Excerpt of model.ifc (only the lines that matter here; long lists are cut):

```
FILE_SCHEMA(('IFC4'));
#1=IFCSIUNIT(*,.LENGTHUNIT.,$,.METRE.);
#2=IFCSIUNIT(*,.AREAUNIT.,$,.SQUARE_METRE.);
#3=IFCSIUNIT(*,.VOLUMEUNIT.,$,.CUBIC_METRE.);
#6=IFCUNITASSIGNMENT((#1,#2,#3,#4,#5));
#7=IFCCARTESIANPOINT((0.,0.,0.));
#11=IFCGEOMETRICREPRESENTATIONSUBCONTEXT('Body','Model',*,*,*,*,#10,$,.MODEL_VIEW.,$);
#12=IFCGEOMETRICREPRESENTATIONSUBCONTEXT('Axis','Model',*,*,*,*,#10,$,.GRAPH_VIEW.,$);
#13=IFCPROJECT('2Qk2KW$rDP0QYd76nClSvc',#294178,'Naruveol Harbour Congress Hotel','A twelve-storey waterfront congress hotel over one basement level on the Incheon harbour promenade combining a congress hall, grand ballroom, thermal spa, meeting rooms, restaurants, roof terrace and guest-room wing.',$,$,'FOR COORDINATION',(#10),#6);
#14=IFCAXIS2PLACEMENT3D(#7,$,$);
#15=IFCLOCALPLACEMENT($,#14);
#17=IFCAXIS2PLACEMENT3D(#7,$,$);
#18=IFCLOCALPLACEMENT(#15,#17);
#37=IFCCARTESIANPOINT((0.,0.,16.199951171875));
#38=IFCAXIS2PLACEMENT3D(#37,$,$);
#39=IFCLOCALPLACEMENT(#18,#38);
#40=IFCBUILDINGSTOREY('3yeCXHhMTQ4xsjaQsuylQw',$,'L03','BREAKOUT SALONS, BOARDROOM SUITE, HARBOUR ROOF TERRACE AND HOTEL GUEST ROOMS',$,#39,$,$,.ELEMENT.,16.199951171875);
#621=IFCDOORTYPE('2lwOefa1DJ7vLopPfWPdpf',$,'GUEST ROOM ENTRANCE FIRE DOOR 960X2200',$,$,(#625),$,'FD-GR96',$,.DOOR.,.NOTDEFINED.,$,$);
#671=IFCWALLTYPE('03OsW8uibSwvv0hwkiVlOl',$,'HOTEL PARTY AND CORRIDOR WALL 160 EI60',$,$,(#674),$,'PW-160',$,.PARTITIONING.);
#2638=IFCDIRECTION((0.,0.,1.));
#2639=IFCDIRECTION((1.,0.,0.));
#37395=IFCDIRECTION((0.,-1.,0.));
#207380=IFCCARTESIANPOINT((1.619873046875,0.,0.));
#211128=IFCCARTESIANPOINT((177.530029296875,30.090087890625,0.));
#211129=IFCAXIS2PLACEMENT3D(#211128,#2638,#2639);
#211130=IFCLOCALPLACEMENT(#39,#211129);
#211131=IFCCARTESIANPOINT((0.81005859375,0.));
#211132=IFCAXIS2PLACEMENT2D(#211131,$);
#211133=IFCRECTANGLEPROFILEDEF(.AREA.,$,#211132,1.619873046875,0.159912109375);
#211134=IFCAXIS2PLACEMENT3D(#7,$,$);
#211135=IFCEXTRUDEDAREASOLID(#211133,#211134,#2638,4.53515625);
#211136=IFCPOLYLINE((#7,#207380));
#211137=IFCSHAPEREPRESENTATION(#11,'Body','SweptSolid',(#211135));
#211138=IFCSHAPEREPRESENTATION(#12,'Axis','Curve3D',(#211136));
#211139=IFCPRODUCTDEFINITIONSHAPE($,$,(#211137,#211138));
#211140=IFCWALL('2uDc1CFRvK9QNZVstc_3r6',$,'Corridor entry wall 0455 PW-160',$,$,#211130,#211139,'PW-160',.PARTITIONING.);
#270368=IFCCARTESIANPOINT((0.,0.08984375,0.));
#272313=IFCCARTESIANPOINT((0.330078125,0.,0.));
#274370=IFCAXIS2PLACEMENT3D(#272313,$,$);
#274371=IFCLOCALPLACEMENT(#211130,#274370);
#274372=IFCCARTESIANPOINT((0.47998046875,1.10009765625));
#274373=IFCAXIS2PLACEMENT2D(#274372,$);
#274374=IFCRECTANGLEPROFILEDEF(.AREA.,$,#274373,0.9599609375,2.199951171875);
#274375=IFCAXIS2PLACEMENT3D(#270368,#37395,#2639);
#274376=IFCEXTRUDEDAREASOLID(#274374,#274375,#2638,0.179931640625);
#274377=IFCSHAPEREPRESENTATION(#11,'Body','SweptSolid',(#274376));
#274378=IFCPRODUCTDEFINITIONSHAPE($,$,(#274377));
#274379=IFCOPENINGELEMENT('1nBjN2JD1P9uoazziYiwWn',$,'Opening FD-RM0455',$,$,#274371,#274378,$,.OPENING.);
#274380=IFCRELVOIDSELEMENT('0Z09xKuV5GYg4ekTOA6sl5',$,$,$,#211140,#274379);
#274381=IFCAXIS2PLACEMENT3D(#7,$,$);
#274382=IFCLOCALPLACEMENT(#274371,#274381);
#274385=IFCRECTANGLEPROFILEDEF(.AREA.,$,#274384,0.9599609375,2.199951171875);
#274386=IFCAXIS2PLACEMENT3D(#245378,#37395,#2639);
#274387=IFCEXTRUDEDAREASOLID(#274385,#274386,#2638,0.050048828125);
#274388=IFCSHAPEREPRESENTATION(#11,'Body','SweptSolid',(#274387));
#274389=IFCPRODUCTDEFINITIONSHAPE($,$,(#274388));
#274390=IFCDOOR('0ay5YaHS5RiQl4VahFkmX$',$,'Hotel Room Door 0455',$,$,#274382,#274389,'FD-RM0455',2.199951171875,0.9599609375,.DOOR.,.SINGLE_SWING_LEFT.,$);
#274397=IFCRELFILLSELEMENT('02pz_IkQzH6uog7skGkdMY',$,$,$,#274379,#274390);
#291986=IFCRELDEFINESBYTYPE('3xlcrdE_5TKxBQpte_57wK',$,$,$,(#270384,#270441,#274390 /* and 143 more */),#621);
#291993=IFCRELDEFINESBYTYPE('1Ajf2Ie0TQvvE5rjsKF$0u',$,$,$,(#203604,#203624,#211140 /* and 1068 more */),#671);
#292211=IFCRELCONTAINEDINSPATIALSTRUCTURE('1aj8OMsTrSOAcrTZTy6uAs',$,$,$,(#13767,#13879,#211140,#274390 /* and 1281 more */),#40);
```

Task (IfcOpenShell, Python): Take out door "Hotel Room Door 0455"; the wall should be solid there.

```python
import ifcopenshell
import ifcopenshell.api.feature
import ifcopenshell.api.root
import ifcopenshell.geom
import ifcopenshell.util.shape

model = ifcopenshell.open("model.ifc")
settings = ifcopenshell.geom.settings()


def volume(element):
    """Net volume in cubic metres, openings subtracted."""
    shape = ifcopenshell.geom.create_shape(settings, element)
    return ifcopenshell.util.shape.get_volume(shape.geometry)


door = model.by_id(274390)
opening = door.FillsVoids[0].RelatingOpeningElement
wall = opening.VoidsElements[0].RelatingBuildingElement
before = volume(wall)

ifcopenshell.api.root.remove_product(model, product=door)
ifcopenshell.api.feature.remove_feature(model, feature=opening)

after = volume(wall)

print(f"wall volume {before:.3f} -> {after:.3f} m3")

model.write("model_edited.ifc")
```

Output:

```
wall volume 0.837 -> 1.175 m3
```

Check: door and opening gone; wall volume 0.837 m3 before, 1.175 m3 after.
